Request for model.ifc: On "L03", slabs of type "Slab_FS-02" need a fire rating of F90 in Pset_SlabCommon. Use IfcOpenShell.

First a look at what the model holds.

```python
import ifcopenshell
import ifcopenshell.util.element

model = ifcopenshell.open("model.ifc")
print(model.schema)
storey = next(s for s in model.by_type("IfcBuildingStorey") if s.Name == "L03")
slabs = [e for e in ifcopenshell.util.element.get_decomposition(storey) if e.is_a("IfcSlab")]
seen = {}
for e in slabs:
    element_type = ifcopenshell.util.element.get_type(e)
    key = (element_type.Name if element_type != e and element_type else None, ifcopenshell.util.element.get_pset(e, "Pset_SlabCommon", "FireRating"))
    seen[key] = seen.get(key, 0) + 1
for (name, value), count in sorted(seen.items(), key=str):
    print(count, "x", name, "|", value)
```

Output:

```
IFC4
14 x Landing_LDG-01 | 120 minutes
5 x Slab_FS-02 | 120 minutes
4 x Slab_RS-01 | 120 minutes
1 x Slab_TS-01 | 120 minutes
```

```python
import ifcopenshell
import ifcopenshell.api.pset
import ifcopenshell.util.element

model = ifcopenshell.open("model.ifc")

storey = next(s for s in model.by_type("IfcBuildingStorey") if s.Name == "L03")
slabs = [e for e in ifcopenshell.util.element.get_decomposition(storey) if e.is_a("IfcSlab")]

count = 0
for e in slabs:
    element_type = ifcopenshell.util.element.get_type(e)
    if element_type in (None, e) or element_type.Name != "Slab_FS-02":
        continue
    # add_pset returns the element's existing set when there is one.
    pset = ifcopenshell.api.pset.add_pset(model, product=e, name="Pset_SlabCommon")
    ifcopenshell.api.pset.edit_pset(model, pset=pset, properties={"FireRating": "F90"})
    count += 1

print(count, "slabs updated")

model.write("model-out.ifc")
```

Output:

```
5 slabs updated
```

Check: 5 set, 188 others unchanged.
